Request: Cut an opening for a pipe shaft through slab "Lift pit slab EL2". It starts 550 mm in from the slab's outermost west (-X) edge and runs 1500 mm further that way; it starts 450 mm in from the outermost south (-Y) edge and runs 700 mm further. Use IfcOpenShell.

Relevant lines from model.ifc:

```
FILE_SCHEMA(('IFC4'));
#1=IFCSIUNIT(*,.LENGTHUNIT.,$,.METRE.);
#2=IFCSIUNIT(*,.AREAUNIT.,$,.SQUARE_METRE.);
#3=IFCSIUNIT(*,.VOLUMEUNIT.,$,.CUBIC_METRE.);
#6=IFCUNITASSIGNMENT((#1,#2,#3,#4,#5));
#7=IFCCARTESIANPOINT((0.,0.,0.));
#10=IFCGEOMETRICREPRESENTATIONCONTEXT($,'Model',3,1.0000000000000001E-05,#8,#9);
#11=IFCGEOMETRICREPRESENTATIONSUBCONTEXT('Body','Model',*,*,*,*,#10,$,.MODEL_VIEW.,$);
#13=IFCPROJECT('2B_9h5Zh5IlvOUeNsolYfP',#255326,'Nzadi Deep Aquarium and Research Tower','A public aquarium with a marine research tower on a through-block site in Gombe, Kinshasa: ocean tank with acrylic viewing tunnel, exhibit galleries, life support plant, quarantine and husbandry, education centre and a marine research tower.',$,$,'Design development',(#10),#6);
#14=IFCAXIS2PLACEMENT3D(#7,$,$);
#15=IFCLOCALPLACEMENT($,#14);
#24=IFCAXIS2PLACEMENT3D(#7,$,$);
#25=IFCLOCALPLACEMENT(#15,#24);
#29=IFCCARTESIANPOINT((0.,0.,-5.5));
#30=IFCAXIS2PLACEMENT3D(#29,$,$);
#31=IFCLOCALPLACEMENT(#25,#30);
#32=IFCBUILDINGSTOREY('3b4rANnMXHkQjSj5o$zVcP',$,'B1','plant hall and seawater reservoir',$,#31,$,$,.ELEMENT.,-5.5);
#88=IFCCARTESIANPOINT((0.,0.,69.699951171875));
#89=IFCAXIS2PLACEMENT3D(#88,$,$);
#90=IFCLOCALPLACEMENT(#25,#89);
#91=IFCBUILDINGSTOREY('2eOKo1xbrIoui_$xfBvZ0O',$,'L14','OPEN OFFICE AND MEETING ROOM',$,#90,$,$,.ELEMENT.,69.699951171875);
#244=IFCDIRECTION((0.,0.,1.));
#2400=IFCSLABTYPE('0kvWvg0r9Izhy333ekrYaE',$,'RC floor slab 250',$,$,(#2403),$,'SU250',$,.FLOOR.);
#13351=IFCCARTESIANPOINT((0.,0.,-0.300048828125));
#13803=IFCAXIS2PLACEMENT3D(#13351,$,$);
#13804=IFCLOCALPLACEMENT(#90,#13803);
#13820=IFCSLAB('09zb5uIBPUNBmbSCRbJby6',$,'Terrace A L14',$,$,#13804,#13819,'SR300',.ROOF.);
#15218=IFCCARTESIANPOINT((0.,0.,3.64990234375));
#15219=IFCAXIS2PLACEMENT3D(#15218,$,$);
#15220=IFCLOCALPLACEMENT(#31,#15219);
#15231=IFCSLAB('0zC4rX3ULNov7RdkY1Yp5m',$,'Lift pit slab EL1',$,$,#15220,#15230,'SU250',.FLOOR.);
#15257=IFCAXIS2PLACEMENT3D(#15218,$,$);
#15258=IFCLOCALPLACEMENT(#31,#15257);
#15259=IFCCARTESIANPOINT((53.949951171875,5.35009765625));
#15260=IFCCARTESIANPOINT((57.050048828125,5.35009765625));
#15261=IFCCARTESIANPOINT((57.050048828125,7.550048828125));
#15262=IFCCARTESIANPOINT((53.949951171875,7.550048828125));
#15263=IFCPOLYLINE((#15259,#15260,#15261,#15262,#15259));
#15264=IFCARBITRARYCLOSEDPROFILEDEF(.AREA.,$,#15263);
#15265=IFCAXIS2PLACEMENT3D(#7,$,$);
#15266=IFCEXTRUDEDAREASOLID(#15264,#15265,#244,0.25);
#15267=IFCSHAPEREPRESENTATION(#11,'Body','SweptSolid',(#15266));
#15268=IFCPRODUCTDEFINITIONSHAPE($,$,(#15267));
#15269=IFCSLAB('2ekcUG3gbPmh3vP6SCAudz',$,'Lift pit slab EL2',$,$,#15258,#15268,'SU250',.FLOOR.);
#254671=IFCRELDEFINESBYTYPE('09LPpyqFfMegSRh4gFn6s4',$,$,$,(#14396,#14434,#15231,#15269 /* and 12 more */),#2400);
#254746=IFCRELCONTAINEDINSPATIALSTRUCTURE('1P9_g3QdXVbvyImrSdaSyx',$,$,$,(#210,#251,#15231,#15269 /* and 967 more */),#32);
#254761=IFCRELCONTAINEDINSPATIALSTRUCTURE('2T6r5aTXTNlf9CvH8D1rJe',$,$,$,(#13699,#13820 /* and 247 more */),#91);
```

```python
import numpy as np
import ifcopenshell
import ifcopenshell.api.feature
import ifcopenshell.api.geometry
import ifcopenshell.api.root
import ifcopenshell.geom
import ifcopenshell.util.placement
import ifcopenshell.util.representation
import ifcopenshell.util.shape
import ifcopenshell.util.unit

model = ifcopenshell.open("model.ifc")
unit_scale = ifcopenshell.util.unit.calculate_unit_scale(model)
settings = ifcopenshell.geom.settings()


def volume(element):
    """Net volume in cubic metres, openings subtracted."""
    shape = ifcopenshell.geom.create_shape(settings, element)
    return ifcopenshell.util.shape.get_volume(shape.geometry)


slab = model.by_id(15269)
before = volume(slab)

# Extent in the slab's own axes, in metres. The edges named are its -X and -Y sides.
slab_shape = ifcopenshell.geom.create_shape(settings, slab)
vertices = ifcopenshell.util.shape.get_vertices(slab_shape.geometry)
x_min, y_min, bottom = vertices.min(axis=0)
top = vertices[:, 2].max()

opening = ifcopenshell.api.root.create_entity(model, ifc_class="IfcOpeningElement", name="Pipe shaft opening", predefined_type="OPENING")
context = ifcopenshell.util.representation.get_context(model, "Model", "Body", "MODEL_VIEW")
width, depth = 1.5, 0.7
outline = [(0.0, 0.0), (width, 0.0), (width, depth), (0.0, depth), (0.0, 0.0)]
# Overshoot both faces by 50 mm so the cut is clean.
shape = ifcopenshell.api.geometry.add_slab_representation(
    model, context=context, depth=top - bottom + 0.1, polyline=outline
)
ifcopenshell.api.geometry.assign_representation(model, product=opening, representation=shape)

matrix = ifcopenshell.util.placement.get_local_placement(slab.ObjectPlacement)
matrix[:, 3] = matrix @ np.append(np.array([x_min + 0.55, y_min + 0.45, bottom - 0.05]) / unit_scale, 1.0)
ifcopenshell.api.geometry.edit_object_placement(model, product=opening, matrix=matrix, is_si=False)
ifcopenshell.api.feature.add_feature(model, feature=opening, element=slab)

after = volume(slab)

print(f"slab volume {before:.3f} -> {after:.3f} m3")

model.write("model_rev.ifc")
```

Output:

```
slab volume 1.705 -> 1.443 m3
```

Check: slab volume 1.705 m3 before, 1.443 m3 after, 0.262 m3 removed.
